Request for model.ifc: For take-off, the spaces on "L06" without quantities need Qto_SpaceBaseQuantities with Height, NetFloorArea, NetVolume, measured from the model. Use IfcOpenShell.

First a look at what the model holds.

```python
import ifcopenshell
import ifcopenshell.util.element
import ifcopenshell.util.unit

model = ifcopenshell.open("model.ifc")
print(model.schema)
for unit_type in ("LENGTHUNIT", "AREAUNIT", "VOLUMEUNIT"):
    print(unit_type, ifcopenshell.util.unit.calculate_unit_scale(model, unit_type))
storey = next(s for s in model.by_type("IfcBuildingStorey") if s.Name == "L06")
spaces = [e for e in ifcopenshell.util.element.get_decomposition(storey) if e.is_a("IfcSpace")]
for e in sorted(spaces, key=lambda e: e.id()):
    print(e.id(), e.is_a(), e.Name, list(ifcopenshell.util.element.get_psets(e, qtos_only=True)), sep=" | ")
```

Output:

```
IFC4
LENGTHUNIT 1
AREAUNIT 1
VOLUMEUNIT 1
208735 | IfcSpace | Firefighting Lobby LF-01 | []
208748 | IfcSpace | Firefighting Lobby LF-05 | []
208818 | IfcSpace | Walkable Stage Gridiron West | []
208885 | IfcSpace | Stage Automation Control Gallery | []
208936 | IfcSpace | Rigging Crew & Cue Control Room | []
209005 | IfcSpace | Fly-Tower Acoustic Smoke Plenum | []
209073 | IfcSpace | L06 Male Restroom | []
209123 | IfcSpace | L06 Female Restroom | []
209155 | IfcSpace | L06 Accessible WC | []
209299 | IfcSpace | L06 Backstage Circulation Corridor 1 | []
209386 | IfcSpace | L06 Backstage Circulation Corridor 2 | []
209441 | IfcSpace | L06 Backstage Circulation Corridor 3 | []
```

```python
import ifcopenshell
import ifcopenshell.api.pset
import ifcopenshell.geom
import ifcopenshell.util.element
import ifcopenshell.util.shape
import ifcopenshell.util.unit

model = ifcopenshell.open("model.ifc")
unit_scale = ifcopenshell.util.unit.calculate_unit_scale(model)
area_scale = ifcopenshell.util.unit.calculate_unit_scale(model, "AREAUNIT")
volume_scale = ifcopenshell.util.unit.calculate_unit_scale(model, "VOLUMEUNIT")
settings = ifcopenshell.geom.settings()

storey = next(s for s in model.by_type("IfcBuildingStorey") if s.Name == "L06")
spaces = [e for e in ifcopenshell.util.element.get_decomposition(storey) if e.is_a("IfcSpace")]

for e in sorted(spaces, key=lambda e: e.id()):
    if ifcopenshell.util.element.get_psets(e, qtos_only=True, should_inherit=False):
        continue
    # Geometry comes back in metres, in the element's own axes.
    shape = ifcopenshell.geom.create_shape(settings, e)
    values = {
        "Height": ifcopenshell.util.shape.get_z(shape.geometry) / unit_scale,
        "NetFloorArea": ifcopenshell.util.shape.get_footprint_area(shape.geometry) / area_scale,
        "NetVolume": ifcopenshell.util.shape.get_volume(shape.geometry) / volume_scale,
    }
    qto = ifcopenshell.api.pset.add_qto(model, product=e, name="Qto_SpaceBaseQuantities")
    ifcopenshell.api.pset.edit_qto(model, qto=qto, properties=values)
    print(e.id(), {k: round(v, 3) for k, v in values.items()})

model.write("model_v2.ifc")
```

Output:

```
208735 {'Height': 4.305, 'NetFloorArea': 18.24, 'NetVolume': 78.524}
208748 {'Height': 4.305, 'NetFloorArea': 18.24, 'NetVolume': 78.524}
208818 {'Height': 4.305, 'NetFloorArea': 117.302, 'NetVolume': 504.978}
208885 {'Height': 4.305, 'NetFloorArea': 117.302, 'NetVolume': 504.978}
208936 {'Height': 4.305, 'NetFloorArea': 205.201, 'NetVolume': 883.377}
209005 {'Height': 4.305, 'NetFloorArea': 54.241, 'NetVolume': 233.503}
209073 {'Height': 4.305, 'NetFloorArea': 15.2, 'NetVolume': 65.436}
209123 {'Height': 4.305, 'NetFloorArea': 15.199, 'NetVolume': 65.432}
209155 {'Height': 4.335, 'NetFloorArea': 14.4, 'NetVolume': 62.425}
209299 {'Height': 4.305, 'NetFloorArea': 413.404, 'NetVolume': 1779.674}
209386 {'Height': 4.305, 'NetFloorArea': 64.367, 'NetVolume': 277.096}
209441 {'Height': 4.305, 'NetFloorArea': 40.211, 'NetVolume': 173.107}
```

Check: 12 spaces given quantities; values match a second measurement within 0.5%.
